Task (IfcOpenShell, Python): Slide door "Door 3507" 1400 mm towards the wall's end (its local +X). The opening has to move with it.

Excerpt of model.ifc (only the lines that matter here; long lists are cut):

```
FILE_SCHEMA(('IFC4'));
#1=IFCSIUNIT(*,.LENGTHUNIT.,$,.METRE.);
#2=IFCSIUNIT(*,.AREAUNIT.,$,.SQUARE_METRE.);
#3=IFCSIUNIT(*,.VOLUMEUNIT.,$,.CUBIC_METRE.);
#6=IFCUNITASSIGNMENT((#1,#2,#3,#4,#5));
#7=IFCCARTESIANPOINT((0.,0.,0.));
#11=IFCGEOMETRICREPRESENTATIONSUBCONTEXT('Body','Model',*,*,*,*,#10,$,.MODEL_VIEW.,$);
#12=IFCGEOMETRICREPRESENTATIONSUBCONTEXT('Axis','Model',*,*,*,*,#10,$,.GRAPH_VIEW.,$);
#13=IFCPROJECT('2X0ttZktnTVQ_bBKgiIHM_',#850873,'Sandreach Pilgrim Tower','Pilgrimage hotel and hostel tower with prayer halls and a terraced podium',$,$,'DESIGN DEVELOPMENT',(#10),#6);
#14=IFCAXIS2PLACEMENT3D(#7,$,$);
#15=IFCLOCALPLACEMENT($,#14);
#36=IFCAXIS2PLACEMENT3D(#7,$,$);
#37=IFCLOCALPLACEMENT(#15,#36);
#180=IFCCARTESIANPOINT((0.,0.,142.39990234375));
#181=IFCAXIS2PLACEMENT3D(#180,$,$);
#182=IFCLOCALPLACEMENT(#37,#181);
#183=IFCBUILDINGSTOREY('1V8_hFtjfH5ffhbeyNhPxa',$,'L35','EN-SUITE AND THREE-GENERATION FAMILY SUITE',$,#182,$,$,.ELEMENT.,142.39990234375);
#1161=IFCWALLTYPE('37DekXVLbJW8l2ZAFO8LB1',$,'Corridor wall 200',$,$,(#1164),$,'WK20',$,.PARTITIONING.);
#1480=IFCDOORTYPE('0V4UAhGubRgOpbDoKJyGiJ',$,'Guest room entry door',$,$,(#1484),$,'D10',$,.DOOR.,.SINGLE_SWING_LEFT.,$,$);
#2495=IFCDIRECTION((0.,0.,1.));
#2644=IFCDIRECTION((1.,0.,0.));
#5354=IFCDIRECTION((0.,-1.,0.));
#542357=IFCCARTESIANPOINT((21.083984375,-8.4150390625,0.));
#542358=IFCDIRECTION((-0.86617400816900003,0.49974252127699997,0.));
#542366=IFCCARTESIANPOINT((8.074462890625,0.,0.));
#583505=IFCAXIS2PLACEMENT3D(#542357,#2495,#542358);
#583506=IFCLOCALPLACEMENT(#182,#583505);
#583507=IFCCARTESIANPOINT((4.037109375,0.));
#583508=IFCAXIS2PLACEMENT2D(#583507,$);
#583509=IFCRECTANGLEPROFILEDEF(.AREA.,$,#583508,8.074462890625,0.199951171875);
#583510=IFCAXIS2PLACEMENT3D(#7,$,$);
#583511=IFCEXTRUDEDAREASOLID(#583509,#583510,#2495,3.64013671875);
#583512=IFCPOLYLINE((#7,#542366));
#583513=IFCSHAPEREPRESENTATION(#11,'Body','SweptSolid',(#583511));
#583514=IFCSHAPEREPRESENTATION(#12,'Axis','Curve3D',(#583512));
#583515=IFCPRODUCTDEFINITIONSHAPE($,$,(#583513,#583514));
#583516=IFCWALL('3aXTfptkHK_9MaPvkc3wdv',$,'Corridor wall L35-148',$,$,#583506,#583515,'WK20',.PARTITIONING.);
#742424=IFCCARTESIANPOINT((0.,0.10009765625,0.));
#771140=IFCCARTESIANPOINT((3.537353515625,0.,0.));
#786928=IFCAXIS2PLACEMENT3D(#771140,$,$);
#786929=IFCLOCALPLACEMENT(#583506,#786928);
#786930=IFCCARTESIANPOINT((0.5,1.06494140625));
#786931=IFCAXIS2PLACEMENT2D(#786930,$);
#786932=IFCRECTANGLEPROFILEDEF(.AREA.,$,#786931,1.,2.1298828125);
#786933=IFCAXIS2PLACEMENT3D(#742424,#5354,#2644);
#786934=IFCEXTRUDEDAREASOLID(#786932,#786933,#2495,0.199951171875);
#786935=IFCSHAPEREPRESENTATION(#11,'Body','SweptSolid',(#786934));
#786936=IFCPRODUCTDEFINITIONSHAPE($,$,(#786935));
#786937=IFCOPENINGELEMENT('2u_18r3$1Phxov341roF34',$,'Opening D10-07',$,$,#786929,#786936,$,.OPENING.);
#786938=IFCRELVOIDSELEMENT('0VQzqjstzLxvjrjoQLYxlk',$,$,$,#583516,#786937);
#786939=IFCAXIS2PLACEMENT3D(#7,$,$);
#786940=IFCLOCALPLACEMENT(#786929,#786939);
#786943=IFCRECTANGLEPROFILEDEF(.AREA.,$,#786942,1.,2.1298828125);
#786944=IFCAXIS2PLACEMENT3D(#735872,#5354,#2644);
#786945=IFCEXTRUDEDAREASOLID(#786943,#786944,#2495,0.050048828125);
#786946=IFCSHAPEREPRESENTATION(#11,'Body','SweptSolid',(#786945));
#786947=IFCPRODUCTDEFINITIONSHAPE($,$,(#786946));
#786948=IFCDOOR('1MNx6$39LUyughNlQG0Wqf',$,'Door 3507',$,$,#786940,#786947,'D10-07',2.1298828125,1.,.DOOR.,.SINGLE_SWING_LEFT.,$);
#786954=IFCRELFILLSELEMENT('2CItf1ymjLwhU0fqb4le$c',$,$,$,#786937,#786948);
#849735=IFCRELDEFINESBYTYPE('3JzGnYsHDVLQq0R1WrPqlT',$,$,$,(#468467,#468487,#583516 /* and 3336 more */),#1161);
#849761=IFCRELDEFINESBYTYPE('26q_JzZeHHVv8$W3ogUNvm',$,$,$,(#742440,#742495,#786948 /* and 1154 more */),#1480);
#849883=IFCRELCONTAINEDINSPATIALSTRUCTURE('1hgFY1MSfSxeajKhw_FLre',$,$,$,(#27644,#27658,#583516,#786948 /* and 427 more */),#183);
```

```python
import ifcopenshell
import ifcopenshell.api.geometry
import ifcopenshell.util.placement

model = ifcopenshell.open("model.ifc")

door = model.by_guid("1MNx6$39LUyughNlQG0Wqf")
opening = door.FillsVoids[0].RelatingOpeningElement
wall = opening.VoidsElements[0].RelatingBuildingElement

wall_matrix = ifcopenshell.util.placement.get_local_placement(wall.ObjectPlacement)
shift = wall_matrix[:3, 0] * 1.4
before = ifcopenshell.util.placement.get_local_placement(door.ObjectPlacement)[:3, 3].copy()

# The door is placed relative to its opening, so it follows when the opening moves.
matrix = ifcopenshell.util.placement.get_local_placement(opening.ObjectPlacement)
matrix[:3, 3] += shift
ifcopenshell.api.geometry.edit_object_placement(
    model, product=opening, matrix=matrix, is_si=False, should_transform_children=True
)

after = ifcopenshell.util.placement.get_local_placement(door.ObjectPlacement)[:3, 3]
print("door moved by", (after - before).round(3) + 0.0)

model.write("model_edited.ifc")
```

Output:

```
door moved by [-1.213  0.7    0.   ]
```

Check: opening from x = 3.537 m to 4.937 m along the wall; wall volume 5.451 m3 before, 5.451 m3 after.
